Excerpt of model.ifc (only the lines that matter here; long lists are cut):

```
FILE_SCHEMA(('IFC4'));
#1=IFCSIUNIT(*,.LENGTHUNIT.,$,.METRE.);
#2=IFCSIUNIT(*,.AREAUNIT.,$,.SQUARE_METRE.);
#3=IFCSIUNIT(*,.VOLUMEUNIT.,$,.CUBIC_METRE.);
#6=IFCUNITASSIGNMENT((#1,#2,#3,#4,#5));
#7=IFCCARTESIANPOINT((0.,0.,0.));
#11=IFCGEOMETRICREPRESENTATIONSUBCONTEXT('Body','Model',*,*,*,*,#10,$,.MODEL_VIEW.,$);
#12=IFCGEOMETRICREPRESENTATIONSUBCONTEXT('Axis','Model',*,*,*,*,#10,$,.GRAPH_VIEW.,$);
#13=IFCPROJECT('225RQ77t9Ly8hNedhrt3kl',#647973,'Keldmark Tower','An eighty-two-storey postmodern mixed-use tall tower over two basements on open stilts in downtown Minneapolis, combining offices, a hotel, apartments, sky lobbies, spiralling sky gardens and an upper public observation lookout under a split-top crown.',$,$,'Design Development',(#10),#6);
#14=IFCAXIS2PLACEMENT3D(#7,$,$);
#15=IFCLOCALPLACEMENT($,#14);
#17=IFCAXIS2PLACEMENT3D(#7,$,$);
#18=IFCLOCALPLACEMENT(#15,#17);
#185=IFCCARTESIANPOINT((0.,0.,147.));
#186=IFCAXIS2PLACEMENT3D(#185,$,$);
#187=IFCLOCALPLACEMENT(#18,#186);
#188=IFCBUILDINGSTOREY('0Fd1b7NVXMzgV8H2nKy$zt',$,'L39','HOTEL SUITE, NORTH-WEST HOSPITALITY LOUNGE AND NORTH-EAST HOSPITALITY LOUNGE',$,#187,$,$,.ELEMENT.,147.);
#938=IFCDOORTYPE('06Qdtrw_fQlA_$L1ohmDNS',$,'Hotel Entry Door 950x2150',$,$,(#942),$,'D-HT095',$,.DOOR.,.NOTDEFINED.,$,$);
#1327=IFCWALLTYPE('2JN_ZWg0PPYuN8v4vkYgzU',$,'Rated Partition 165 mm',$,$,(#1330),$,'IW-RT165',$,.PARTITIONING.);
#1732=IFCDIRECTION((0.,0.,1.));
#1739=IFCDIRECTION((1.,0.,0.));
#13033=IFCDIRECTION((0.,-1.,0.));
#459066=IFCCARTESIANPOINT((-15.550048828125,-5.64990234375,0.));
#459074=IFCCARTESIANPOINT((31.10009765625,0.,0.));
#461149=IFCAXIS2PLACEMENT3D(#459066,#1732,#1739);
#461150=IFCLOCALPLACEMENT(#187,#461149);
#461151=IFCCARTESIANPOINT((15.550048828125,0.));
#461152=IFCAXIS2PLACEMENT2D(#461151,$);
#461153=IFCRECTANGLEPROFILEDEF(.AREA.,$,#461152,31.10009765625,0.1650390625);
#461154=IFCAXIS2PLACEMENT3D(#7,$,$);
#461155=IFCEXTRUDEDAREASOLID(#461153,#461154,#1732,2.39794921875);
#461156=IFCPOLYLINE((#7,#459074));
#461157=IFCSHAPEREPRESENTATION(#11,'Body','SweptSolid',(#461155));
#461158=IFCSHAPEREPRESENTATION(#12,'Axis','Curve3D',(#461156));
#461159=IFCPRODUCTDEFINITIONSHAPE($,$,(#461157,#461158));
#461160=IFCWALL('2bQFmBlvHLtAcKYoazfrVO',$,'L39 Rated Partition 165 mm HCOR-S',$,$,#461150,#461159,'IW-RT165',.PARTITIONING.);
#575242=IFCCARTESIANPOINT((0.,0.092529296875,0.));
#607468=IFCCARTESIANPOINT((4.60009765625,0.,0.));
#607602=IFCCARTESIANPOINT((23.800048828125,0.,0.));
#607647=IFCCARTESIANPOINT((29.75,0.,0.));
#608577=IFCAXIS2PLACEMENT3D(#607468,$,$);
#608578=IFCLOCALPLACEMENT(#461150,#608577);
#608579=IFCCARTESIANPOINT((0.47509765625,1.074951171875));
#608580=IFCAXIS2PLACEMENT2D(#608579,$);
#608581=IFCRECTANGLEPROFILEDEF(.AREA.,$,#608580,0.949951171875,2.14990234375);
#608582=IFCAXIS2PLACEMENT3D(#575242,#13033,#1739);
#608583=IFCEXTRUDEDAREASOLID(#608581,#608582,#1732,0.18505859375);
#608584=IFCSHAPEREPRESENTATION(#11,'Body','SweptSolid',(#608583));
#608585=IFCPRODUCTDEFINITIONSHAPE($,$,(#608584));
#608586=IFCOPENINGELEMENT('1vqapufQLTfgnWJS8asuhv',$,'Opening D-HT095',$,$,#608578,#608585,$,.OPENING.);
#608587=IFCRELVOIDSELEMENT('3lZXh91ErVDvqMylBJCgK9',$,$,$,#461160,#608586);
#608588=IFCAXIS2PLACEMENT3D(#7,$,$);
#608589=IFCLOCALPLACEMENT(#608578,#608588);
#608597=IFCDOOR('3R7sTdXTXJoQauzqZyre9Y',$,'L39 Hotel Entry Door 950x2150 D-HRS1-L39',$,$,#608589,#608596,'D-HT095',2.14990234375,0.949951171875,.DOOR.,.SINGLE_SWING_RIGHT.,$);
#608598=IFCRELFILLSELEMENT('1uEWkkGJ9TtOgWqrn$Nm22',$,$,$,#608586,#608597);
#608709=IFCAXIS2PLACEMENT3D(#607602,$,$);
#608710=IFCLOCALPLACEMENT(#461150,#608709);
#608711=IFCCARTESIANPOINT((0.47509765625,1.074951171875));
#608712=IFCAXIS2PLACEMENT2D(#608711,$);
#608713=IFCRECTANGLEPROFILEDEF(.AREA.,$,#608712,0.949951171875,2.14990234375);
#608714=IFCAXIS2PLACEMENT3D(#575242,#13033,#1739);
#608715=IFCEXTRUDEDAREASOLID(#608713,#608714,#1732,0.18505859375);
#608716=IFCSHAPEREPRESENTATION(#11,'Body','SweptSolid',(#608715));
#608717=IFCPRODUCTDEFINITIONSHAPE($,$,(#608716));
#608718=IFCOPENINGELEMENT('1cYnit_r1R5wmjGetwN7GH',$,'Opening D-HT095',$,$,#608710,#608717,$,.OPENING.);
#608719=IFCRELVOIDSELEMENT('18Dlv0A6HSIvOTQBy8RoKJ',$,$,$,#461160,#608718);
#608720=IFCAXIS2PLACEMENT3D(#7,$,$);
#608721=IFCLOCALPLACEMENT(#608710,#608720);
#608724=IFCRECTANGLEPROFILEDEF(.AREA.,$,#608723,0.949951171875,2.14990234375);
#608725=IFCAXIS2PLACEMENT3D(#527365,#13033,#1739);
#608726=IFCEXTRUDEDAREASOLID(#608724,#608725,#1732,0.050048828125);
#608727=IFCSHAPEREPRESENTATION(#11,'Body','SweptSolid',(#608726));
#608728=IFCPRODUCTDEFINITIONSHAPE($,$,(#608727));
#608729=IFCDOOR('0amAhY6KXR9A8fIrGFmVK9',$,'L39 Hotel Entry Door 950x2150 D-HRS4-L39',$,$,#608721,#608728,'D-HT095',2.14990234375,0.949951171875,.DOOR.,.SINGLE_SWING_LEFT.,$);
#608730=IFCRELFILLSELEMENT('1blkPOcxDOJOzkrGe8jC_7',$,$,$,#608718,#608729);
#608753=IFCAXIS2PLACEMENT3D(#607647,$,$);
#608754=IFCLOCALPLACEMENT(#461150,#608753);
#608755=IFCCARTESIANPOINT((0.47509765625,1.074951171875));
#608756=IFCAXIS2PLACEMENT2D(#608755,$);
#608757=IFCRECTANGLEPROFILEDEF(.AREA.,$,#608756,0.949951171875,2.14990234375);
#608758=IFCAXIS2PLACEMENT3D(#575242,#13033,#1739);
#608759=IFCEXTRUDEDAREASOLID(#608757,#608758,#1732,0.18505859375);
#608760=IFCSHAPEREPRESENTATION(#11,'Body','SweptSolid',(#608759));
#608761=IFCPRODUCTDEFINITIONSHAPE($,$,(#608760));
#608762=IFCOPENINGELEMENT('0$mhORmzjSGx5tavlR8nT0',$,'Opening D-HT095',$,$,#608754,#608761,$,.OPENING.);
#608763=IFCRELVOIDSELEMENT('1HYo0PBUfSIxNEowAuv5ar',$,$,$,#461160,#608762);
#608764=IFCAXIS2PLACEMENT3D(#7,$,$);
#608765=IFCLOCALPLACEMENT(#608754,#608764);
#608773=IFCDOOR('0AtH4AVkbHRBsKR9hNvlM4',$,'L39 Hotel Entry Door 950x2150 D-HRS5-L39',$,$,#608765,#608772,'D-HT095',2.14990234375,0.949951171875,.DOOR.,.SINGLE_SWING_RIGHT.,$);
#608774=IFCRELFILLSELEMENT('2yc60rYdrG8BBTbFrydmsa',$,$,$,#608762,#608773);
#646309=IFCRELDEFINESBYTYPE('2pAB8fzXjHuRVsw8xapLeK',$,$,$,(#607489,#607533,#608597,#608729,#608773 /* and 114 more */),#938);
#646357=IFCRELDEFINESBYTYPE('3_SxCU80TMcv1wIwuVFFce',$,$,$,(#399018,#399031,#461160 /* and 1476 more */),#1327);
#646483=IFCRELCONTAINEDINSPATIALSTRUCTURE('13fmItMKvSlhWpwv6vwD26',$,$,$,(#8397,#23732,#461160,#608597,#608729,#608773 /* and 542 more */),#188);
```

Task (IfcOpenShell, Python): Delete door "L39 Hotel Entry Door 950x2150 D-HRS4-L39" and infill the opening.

```python
import ifcopenshell
import ifcopenshell.api.feature
import ifcopenshell.api.root
import ifcopenshell.geom
import ifcopenshell.util.shape

model = ifcopenshell.open("model.ifc")
settings = ifcopenshell.geom.settings()


def volume(element):
    """Net volume in cubic metres, openings subtracted."""
    shape = ifcopenshell.geom.create_shape(settings, element)
    return ifcopenshell.util.shape.get_volume(shape.geometry)


door = model.by_id(608729)
opening = door.FillsVoids[0].RelatingOpeningElement
wall = opening.VoidsElements[0].RelatingBuildingElement
before = volume(wall)

ifcopenshell.api.root.remove_product(model, product=door)
ifcopenshell.api.feature.remove_feature(model, feature=opening)

after = volume(wall)

print(f"wall volume {before:.3f} -> {after:.3f} m3")

model.write("model_rev.ifc")
```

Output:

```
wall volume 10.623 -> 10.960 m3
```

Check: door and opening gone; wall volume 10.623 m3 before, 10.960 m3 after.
